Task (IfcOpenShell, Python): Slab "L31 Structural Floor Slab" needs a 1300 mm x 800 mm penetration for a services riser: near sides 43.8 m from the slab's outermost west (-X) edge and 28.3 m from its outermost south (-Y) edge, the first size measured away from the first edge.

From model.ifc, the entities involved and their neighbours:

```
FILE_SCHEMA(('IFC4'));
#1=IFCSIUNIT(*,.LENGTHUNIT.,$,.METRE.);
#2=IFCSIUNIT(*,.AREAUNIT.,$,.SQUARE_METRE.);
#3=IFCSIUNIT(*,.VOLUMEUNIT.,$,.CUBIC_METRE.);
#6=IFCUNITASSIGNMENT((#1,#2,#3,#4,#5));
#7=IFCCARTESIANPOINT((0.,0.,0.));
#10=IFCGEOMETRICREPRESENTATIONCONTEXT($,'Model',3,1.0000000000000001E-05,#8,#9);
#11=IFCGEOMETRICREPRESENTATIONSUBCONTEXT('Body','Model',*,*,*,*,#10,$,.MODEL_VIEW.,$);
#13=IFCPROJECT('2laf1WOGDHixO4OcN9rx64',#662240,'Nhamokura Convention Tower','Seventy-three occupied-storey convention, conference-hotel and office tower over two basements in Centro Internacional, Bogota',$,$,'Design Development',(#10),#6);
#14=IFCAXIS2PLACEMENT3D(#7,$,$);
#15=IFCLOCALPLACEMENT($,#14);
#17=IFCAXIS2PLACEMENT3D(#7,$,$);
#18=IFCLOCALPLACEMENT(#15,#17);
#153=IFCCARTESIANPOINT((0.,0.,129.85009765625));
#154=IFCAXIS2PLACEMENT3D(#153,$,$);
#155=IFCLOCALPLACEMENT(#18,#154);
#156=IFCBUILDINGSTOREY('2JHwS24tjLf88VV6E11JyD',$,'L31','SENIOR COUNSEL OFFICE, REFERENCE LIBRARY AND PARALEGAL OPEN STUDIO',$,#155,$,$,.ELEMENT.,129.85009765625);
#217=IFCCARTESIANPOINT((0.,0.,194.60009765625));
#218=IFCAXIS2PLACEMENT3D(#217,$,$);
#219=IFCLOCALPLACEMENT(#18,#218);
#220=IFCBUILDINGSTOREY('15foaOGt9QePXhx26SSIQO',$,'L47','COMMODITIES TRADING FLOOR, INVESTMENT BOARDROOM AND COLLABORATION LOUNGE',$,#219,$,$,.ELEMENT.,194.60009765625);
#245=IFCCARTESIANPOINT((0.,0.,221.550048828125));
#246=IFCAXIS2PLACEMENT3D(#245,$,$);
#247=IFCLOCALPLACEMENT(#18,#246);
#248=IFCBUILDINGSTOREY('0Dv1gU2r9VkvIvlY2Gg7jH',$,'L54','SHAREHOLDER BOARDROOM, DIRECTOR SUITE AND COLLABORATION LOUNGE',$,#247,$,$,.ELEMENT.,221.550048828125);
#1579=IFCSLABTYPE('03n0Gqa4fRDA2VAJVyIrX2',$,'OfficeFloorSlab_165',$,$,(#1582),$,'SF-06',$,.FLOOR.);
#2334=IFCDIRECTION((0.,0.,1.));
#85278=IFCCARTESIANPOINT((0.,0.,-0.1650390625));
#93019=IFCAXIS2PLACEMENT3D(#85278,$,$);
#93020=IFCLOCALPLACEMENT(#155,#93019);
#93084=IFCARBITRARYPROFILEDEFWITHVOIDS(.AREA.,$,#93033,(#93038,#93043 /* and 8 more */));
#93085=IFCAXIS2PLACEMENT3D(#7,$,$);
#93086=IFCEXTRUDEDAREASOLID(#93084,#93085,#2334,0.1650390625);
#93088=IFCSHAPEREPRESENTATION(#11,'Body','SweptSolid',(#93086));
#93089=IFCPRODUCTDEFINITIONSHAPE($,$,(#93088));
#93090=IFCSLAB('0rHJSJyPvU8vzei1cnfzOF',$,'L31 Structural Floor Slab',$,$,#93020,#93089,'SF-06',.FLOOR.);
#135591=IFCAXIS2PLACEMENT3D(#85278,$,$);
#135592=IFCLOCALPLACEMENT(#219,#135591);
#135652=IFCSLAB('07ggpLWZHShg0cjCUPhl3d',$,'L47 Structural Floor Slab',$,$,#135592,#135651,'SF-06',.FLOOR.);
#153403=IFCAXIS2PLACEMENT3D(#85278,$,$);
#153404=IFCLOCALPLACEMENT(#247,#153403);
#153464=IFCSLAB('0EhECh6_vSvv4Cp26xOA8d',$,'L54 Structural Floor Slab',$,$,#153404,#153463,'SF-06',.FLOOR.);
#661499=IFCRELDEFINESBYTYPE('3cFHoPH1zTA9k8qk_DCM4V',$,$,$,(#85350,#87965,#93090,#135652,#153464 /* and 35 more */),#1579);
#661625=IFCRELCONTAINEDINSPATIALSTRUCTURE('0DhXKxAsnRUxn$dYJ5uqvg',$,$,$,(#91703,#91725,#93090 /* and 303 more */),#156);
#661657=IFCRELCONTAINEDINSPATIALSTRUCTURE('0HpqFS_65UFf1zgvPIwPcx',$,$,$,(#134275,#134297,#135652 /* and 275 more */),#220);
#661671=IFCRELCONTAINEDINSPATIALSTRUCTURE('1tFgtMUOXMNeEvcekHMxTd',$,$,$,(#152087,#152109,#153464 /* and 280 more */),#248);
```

```python
import numpy as np
import ifcopenshell
import ifcopenshell.api.feature
import ifcopenshell.api.geometry
import ifcopenshell.api.root
import ifcopenshell.geom
import ifcopenshell.util.placement
import ifcopenshell.util.representation
import ifcopenshell.util.shape
import ifcopenshell.util.unit

model = ifcopenshell.open("model.ifc")
unit_scale = ifcopenshell.util.unit.calculate_unit_scale(model)
settings = ifcopenshell.geom.settings()


def volume(element):
    """Net volume in cubic metres, openings subtracted."""
    shape = ifcopenshell.geom.create_shape(settings, element)
    return ifcopenshell.util.shape.get_volume(shape.geometry)


slab = model.by_id(93090)
before = volume(slab)

# Extent in the slab's own axes, in metres. The edges named are its -X and -Y sides.
slab_shape = ifcopenshell.geom.create_shape(settings, slab)
vertices = ifcopenshell.util.shape.get_vertices(slab_shape.geometry)
x_min, y_min, bottom = vertices.min(axis=0)
top = vertices[:, 2].max()

opening = ifcopenshell.api.root.create_entity(model, ifc_class="IfcOpeningElement", name="Services riser opening", predefined_type="OPENING")
context = ifcopenshell.util.representation.get_context(model, "Model", "Body", "MODEL_VIEW")
width, depth = 1.3, 0.8
outline = [(0.0, 0.0), (width, 0.0), (width, depth), (0.0, depth), (0.0, 0.0)]
# Overshoot both faces by 50 mm so the cut is clean.
shape = ifcopenshell.api.geometry.add_slab_representation(
    model, context=context, depth=top - bottom + 0.1, polyline=outline
)
ifcopenshell.api.geometry.assign_representation(model, product=opening, representation=shape)

matrix = ifcopenshell.util.placement.get_local_placement(slab.ObjectPlacement)
matrix[:, 3] = matrix @ np.append(np.array([x_min + 43.8, y_min + 28.3, bottom - 0.05]) / unit_scale, 1.0)
ifcopenshell.api.geometry.edit_object_placement(model, product=opening, matrix=matrix, is_si=False)
ifcopenshell.api.feature.add_feature(model, feature=opening, element=slab)

after = volume(slab)

print(f"slab volume {before:.3f} -> {after:.3f} m3")

model.write("model-out.ifc")
```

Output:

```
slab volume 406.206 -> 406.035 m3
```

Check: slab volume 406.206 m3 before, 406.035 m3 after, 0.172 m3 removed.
